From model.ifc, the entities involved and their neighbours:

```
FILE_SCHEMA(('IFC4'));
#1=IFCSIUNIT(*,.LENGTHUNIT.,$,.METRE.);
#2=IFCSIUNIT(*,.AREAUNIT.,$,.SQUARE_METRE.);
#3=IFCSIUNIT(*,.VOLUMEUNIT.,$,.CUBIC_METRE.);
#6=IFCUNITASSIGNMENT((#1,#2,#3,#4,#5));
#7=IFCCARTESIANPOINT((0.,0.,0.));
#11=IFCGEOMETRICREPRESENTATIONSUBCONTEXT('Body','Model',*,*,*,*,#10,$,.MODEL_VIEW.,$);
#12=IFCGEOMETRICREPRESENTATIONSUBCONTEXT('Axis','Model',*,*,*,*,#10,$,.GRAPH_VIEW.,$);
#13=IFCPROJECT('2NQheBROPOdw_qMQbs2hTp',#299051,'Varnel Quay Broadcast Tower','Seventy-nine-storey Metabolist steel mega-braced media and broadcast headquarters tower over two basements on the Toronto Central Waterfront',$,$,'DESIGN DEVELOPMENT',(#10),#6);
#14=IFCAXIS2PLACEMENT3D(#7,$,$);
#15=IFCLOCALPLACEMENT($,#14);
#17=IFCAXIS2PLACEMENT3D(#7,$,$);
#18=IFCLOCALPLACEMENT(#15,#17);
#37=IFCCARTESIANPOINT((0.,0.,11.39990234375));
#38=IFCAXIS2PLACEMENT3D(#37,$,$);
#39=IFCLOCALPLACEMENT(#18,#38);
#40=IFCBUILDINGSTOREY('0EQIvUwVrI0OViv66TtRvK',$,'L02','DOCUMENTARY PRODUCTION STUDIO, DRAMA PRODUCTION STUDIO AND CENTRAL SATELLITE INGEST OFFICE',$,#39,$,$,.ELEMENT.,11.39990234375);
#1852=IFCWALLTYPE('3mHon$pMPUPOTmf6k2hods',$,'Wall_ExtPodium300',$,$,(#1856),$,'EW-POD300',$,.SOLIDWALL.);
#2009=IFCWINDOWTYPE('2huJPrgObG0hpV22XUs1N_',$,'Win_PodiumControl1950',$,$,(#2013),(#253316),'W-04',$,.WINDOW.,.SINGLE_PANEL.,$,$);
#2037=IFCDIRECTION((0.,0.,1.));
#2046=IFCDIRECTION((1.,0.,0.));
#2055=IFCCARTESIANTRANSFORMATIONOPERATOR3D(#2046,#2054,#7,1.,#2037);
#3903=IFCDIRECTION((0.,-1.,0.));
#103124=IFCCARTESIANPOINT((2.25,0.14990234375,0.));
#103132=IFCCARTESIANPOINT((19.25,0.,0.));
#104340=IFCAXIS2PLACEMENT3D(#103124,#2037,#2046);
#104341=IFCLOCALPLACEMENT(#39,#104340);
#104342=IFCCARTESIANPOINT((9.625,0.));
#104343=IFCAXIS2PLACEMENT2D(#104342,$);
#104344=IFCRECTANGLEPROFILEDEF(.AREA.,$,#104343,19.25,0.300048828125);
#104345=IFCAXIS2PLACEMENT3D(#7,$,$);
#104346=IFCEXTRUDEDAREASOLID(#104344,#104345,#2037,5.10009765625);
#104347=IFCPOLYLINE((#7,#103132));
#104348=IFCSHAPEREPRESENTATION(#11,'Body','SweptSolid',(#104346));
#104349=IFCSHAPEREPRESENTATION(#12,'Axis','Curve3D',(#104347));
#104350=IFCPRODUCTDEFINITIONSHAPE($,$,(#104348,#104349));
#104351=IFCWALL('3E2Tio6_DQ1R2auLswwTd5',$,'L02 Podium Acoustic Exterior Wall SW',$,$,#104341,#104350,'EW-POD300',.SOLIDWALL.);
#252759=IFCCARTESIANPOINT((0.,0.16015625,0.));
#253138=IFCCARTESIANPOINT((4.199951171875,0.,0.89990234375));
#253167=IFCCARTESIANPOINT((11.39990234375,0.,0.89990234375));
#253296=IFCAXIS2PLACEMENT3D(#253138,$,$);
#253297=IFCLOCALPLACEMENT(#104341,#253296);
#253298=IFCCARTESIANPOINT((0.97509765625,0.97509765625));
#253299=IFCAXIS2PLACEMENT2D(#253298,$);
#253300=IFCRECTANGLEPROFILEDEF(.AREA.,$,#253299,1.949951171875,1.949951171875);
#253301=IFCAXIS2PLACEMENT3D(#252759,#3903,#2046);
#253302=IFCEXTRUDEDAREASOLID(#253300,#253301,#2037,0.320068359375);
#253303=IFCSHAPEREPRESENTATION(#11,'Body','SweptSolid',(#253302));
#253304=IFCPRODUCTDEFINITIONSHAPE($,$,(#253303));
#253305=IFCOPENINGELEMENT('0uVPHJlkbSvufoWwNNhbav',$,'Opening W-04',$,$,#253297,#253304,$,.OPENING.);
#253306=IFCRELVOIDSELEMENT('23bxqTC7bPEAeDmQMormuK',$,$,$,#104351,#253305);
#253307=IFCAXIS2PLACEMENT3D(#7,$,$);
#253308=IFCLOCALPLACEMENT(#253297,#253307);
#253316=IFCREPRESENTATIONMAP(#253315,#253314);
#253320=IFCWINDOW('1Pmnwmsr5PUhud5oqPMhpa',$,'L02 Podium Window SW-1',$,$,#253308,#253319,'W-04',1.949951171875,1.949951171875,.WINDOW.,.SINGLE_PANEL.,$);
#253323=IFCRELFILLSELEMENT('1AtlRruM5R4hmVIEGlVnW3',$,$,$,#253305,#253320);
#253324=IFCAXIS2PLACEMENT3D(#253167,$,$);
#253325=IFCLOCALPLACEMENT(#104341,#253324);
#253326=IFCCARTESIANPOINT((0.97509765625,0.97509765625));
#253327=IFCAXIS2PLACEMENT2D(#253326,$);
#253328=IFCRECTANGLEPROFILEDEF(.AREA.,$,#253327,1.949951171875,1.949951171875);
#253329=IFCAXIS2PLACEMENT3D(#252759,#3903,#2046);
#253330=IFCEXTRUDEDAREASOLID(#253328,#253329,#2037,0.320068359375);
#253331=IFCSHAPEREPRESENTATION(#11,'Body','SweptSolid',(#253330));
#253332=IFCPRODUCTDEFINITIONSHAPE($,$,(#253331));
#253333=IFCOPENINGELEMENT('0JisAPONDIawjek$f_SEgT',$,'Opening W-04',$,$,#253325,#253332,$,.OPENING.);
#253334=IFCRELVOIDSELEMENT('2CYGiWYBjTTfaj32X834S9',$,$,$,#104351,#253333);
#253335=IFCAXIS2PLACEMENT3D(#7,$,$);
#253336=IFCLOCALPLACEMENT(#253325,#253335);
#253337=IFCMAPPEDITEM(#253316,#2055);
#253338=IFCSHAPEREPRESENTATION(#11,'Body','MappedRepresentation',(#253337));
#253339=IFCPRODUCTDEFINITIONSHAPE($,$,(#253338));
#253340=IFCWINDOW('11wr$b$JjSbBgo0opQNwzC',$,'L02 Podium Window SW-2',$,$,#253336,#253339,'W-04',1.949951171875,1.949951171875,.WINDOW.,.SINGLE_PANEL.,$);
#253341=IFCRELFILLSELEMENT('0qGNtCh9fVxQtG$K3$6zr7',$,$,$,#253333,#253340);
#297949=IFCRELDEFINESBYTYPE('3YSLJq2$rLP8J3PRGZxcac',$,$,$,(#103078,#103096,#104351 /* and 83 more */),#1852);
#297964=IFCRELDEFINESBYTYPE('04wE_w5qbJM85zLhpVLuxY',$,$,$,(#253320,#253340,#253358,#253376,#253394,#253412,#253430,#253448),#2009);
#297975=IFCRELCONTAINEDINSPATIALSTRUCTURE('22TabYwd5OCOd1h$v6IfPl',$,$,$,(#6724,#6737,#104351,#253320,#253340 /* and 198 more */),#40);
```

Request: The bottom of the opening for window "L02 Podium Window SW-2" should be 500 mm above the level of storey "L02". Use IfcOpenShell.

```python
import numpy as np
import ifcopenshell
import ifcopenshell.api.geometry
import ifcopenshell.geom
import ifcopenshell.util.element
import ifcopenshell.util.placement
import ifcopenshell.util.shape
import ifcopenshell.util.unit

model = ifcopenshell.open("model.ifc")
unit_scale = ifcopenshell.util.unit.calculate_unit_scale(model)

window = model.by_guid("11wr$b$JjSbBgo0opQNwzC")
opening = window.FillsVoids[0].RelatingOpeningElement
storey = ifcopenshell.util.element.get_container(window, ifc_class="IfcBuildingStorey")
level = ifcopenshell.util.placement.get_local_placement(storey.ObjectPlacement)[2, 3]

# The opening's origin need not be at the sill, so measure its lowest point.
shape = ifcopenshell.geom.create_shape(ifcopenshell.geom.settings(), opening)
bottom = ifcopenshell.util.shape.get_shape_bottom_elevation(shape, shape.geometry) / unit_scale
dz = level + 0.5 / unit_scale - bottom

shift = np.array([0.0, 0.0, dz])
# The window is placed relative to its opening, so it follows when the opening moves.
matrix = ifcopenshell.util.placement.get_local_placement(opening.ObjectPlacement)
matrix[:3, 3] += shift
ifcopenshell.api.geometry.edit_object_placement(
    model, product=opening, matrix=matrix, is_si=False, should_transform_children=True
)

print(f"moved by {dz * unit_scale:+.3f} m")

model.write("model_updated.ifc")
```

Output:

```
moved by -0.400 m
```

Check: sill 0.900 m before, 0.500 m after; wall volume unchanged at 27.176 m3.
